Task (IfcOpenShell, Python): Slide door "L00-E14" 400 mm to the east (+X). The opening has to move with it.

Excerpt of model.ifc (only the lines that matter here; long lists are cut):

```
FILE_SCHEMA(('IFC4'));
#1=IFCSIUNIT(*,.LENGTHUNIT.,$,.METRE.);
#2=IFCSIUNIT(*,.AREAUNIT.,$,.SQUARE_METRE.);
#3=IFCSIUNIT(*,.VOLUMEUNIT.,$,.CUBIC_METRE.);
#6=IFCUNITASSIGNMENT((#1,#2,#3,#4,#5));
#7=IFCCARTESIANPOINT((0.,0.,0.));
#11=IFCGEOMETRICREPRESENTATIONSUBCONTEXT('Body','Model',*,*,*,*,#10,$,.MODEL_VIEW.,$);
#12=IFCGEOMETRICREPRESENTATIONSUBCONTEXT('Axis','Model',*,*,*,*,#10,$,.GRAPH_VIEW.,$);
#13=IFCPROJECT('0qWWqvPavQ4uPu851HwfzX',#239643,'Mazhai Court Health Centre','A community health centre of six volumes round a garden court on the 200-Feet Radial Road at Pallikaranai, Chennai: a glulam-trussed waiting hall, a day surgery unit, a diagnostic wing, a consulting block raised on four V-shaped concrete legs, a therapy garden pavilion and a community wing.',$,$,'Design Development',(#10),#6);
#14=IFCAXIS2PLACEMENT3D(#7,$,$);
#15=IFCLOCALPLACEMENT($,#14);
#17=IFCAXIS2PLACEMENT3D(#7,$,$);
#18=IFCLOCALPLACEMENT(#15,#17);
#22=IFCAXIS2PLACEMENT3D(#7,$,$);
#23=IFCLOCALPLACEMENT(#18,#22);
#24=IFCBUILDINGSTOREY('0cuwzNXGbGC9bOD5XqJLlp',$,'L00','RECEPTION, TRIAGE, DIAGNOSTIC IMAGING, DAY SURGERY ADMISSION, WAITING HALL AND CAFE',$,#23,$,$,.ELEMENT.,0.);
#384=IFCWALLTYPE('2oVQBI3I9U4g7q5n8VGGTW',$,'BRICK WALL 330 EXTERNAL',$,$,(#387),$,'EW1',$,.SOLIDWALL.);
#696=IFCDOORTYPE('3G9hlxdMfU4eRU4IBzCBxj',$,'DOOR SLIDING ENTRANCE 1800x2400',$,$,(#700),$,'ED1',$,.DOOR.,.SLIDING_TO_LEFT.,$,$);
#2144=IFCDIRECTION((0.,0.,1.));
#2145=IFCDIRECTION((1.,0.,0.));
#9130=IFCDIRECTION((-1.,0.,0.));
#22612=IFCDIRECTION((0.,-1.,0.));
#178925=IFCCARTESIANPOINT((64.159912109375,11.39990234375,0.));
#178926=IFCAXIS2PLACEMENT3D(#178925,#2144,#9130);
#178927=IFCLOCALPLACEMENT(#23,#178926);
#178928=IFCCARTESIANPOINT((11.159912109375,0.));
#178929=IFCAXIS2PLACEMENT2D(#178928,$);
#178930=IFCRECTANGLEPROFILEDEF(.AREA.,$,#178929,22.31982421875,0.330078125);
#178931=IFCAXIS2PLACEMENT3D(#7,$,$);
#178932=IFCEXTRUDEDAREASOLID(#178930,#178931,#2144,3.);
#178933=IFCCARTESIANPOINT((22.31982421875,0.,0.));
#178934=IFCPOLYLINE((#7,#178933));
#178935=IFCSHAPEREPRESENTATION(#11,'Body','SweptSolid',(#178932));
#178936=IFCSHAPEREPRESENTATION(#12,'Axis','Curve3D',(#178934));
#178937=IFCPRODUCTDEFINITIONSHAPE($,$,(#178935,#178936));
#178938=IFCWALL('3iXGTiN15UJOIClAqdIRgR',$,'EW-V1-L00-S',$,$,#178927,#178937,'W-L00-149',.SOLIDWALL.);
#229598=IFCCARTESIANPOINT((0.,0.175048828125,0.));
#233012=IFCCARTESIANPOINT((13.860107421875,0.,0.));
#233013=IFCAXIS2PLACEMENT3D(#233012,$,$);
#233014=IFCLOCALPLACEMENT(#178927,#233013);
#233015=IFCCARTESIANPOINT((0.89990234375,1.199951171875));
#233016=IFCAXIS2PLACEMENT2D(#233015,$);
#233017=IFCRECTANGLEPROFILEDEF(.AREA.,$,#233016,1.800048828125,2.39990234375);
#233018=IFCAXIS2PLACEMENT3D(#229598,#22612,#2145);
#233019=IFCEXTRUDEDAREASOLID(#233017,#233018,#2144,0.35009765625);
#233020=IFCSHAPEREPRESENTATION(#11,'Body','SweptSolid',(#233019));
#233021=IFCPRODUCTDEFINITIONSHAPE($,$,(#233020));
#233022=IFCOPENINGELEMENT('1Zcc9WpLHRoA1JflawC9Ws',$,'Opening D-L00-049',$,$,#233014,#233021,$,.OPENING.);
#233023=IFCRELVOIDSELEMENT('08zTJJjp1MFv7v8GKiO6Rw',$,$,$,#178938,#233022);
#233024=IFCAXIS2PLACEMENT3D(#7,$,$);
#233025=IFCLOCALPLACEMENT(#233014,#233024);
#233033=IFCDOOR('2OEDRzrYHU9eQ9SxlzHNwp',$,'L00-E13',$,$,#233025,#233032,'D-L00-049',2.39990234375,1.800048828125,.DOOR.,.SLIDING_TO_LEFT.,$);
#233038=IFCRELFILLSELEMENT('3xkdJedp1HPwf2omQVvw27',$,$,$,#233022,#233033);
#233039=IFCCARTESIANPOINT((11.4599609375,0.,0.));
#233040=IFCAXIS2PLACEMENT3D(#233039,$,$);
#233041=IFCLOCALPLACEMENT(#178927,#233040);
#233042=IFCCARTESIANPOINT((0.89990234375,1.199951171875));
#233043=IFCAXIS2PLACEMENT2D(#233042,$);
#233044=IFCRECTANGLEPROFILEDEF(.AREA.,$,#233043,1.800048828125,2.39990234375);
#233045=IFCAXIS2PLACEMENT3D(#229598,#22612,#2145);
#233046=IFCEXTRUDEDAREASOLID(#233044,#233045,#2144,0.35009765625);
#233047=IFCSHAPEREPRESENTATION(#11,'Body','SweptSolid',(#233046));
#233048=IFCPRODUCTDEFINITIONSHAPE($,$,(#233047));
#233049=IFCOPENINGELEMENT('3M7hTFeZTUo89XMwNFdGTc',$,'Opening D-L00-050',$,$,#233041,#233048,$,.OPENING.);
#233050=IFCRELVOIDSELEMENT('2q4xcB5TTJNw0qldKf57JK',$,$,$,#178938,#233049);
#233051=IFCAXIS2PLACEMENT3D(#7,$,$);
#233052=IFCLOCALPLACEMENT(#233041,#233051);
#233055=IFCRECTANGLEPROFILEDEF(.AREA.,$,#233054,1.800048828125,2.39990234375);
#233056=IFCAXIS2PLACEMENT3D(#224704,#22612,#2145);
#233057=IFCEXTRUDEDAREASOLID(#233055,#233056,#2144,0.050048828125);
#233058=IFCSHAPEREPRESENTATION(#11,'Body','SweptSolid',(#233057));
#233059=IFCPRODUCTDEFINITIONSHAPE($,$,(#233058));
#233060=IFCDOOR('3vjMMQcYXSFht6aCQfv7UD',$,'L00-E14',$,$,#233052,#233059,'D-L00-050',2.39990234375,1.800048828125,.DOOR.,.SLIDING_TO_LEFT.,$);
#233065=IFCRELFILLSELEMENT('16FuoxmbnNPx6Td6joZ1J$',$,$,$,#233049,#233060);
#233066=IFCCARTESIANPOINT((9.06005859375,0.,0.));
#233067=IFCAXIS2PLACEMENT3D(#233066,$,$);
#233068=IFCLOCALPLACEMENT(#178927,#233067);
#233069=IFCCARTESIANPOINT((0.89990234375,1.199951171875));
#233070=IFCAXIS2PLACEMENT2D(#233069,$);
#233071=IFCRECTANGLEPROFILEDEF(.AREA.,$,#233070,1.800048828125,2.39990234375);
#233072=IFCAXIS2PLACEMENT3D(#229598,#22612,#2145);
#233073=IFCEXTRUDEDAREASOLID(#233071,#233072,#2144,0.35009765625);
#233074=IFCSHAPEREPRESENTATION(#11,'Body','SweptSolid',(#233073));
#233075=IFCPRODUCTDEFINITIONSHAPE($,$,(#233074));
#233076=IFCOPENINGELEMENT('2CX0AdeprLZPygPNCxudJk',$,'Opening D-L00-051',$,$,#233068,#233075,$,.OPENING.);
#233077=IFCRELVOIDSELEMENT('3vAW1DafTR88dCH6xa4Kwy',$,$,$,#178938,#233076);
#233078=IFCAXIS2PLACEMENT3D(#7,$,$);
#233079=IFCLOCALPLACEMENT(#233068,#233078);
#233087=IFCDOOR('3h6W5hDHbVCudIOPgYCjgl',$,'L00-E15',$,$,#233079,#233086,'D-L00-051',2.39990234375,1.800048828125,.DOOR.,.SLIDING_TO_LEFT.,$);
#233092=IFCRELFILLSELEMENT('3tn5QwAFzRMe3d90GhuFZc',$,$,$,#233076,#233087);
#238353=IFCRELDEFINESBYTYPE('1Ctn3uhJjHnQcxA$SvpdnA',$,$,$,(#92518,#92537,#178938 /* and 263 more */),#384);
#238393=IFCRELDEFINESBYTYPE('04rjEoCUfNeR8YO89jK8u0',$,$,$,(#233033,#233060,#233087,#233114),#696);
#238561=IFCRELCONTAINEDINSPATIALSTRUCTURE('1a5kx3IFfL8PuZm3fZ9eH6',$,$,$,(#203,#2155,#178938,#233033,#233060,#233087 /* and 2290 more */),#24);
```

```python
import ifcopenshell
import ifcopenshell.api.geometry
import ifcopenshell.util.placement
import ifcopenshell.util.unit

model = ifcopenshell.open("model.ifc")
unit_scale = ifcopenshell.util.unit.calculate_unit_scale(model)

door = model.by_guid("3vjMMQcYXSFht6aCQfv7UD")
opening = door.FillsVoids[0].RelatingOpeningElement
wall = opening.VoidsElements[0].RelatingBuildingElement

wall_matrix = ifcopenshell.util.placement.get_local_placement(wall.ObjectPlacement)
shift = wall_matrix[:3, 0] * -0.4 / unit_scale
before = ifcopenshell.util.placement.get_local_placement(door.ObjectPlacement)[:3, 3].copy()

# The door is placed relative to its opening, so it follows when the opening moves.
matrix = ifcopenshell.util.placement.get_local_placement(opening.ObjectPlacement)
matrix[:3, 3] += shift
ifcopenshell.api.geometry.edit_object_placement(
    model, product=opening, matrix=matrix, is_si=False, should_transform_children=True
)

after = ifcopenshell.util.placement.get_local_placement(door.ObjectPlacement)[:3, 3]
print("door moved by", (after - before).round(3) + 0.0)

model.write("model_edited.ifc")
```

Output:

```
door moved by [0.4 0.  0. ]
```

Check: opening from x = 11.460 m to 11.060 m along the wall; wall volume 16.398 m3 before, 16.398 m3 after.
